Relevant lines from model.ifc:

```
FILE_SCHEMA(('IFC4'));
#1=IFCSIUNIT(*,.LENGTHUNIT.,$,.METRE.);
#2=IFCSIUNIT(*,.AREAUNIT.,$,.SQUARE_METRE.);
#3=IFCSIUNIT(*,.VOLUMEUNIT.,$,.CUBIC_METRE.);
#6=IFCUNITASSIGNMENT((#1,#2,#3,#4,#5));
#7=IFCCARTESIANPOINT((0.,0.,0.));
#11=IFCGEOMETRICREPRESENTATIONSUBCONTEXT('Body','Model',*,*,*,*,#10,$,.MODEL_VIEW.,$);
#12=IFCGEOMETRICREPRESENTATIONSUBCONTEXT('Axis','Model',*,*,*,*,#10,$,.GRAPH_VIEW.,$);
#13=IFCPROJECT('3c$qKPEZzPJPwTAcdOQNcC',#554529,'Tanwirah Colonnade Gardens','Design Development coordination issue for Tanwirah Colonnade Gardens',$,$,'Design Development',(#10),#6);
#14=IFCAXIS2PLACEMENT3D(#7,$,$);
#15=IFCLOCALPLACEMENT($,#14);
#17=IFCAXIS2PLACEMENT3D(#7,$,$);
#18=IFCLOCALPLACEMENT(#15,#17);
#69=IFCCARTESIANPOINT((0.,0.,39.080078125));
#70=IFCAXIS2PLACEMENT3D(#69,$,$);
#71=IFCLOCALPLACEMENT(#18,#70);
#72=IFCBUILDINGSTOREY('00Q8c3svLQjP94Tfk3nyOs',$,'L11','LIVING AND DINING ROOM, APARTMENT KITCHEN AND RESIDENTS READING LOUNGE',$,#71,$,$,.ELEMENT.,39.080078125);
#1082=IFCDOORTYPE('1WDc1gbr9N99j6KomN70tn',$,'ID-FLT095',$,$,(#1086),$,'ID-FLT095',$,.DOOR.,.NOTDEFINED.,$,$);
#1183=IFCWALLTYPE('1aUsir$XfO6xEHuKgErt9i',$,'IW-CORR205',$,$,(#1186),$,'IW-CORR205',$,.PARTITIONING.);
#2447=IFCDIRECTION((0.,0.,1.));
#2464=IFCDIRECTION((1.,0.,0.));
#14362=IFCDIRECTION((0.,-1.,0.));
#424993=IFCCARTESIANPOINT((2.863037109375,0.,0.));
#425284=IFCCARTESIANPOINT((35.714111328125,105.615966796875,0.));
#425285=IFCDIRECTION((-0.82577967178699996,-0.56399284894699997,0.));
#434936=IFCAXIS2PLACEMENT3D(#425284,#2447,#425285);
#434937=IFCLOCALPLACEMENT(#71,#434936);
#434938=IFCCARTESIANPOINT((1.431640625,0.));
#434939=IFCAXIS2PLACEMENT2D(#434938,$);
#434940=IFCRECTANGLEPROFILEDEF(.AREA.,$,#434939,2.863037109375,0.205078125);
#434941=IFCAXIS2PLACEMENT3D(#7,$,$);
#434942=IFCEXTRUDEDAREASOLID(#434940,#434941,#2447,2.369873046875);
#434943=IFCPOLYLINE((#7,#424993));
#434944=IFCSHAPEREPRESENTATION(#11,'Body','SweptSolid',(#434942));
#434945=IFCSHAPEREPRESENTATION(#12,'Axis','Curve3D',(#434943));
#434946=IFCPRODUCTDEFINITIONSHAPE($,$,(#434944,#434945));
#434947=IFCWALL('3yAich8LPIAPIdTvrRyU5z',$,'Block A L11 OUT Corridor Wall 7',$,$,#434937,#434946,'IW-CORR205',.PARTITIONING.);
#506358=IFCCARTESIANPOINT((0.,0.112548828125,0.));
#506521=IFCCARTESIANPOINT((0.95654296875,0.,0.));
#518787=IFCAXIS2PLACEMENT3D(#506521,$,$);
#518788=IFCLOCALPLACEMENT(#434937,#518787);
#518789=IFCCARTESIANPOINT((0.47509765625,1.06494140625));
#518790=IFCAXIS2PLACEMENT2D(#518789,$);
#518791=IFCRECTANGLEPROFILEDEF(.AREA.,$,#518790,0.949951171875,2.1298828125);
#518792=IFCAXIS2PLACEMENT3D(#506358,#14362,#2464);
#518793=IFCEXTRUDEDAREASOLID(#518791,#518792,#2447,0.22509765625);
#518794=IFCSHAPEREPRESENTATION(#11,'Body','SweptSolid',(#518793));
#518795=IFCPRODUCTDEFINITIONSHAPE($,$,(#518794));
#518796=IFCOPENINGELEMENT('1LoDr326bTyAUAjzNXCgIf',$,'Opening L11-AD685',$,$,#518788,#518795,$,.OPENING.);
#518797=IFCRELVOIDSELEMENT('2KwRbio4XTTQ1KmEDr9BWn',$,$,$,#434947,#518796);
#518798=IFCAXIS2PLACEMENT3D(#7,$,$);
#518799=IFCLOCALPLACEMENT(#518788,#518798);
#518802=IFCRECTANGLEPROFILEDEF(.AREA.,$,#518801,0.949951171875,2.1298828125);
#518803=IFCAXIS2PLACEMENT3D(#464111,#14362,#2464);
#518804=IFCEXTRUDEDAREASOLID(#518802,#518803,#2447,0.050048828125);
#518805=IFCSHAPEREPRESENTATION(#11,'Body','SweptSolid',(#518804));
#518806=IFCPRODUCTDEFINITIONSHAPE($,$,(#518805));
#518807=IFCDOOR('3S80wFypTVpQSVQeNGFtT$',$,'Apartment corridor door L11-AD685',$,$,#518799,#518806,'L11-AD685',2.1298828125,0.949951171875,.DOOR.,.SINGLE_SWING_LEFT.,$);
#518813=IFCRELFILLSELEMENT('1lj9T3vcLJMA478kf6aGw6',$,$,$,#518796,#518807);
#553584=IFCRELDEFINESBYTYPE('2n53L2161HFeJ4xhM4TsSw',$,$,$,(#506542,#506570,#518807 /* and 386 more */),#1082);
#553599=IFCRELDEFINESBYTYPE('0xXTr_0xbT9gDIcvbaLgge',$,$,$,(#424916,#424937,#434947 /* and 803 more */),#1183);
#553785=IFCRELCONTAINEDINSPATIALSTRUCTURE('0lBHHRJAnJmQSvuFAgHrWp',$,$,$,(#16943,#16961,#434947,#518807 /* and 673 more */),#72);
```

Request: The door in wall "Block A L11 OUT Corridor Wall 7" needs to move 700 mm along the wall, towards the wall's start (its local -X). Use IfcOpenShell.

```python
import ifcopenshell
import ifcopenshell.api.geometry
import ifcopenshell.util.placement

model = ifcopenshell.open("model.ifc")

door = model.by_id(518807)
opening = door.FillsVoids[0].RelatingOpeningElement
wall = opening.VoidsElements[0].RelatingBuildingElement

wall_matrix = ifcopenshell.util.placement.get_local_placement(wall.ObjectPlacement)
shift = wall_matrix[:3, 0] * -0.7
before = ifcopenshell.util.placement.get_local_placement(door.ObjectPlacement)[:3, 3].copy()

# The door is placed relative to its opening, so it follows when the opening moves.
matrix = ifcopenshell.util.placement.get_local_placement(opening.ObjectPlacement)
matrix[:3, 3] += shift
ifcopenshell.api.geometry.edit_object_placement(
    model, product=opening, matrix=matrix, is_si=False, should_transform_children=True
)

after = ifcopenshell.util.placement.get_local_placement(door.ObjectPlacement)[:3, 3]
print("door moved by", (after - before).round(3) + 0.0)

model.write("model-out.ifc")
```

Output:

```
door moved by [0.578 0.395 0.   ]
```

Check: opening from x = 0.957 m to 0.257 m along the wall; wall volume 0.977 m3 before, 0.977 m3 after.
